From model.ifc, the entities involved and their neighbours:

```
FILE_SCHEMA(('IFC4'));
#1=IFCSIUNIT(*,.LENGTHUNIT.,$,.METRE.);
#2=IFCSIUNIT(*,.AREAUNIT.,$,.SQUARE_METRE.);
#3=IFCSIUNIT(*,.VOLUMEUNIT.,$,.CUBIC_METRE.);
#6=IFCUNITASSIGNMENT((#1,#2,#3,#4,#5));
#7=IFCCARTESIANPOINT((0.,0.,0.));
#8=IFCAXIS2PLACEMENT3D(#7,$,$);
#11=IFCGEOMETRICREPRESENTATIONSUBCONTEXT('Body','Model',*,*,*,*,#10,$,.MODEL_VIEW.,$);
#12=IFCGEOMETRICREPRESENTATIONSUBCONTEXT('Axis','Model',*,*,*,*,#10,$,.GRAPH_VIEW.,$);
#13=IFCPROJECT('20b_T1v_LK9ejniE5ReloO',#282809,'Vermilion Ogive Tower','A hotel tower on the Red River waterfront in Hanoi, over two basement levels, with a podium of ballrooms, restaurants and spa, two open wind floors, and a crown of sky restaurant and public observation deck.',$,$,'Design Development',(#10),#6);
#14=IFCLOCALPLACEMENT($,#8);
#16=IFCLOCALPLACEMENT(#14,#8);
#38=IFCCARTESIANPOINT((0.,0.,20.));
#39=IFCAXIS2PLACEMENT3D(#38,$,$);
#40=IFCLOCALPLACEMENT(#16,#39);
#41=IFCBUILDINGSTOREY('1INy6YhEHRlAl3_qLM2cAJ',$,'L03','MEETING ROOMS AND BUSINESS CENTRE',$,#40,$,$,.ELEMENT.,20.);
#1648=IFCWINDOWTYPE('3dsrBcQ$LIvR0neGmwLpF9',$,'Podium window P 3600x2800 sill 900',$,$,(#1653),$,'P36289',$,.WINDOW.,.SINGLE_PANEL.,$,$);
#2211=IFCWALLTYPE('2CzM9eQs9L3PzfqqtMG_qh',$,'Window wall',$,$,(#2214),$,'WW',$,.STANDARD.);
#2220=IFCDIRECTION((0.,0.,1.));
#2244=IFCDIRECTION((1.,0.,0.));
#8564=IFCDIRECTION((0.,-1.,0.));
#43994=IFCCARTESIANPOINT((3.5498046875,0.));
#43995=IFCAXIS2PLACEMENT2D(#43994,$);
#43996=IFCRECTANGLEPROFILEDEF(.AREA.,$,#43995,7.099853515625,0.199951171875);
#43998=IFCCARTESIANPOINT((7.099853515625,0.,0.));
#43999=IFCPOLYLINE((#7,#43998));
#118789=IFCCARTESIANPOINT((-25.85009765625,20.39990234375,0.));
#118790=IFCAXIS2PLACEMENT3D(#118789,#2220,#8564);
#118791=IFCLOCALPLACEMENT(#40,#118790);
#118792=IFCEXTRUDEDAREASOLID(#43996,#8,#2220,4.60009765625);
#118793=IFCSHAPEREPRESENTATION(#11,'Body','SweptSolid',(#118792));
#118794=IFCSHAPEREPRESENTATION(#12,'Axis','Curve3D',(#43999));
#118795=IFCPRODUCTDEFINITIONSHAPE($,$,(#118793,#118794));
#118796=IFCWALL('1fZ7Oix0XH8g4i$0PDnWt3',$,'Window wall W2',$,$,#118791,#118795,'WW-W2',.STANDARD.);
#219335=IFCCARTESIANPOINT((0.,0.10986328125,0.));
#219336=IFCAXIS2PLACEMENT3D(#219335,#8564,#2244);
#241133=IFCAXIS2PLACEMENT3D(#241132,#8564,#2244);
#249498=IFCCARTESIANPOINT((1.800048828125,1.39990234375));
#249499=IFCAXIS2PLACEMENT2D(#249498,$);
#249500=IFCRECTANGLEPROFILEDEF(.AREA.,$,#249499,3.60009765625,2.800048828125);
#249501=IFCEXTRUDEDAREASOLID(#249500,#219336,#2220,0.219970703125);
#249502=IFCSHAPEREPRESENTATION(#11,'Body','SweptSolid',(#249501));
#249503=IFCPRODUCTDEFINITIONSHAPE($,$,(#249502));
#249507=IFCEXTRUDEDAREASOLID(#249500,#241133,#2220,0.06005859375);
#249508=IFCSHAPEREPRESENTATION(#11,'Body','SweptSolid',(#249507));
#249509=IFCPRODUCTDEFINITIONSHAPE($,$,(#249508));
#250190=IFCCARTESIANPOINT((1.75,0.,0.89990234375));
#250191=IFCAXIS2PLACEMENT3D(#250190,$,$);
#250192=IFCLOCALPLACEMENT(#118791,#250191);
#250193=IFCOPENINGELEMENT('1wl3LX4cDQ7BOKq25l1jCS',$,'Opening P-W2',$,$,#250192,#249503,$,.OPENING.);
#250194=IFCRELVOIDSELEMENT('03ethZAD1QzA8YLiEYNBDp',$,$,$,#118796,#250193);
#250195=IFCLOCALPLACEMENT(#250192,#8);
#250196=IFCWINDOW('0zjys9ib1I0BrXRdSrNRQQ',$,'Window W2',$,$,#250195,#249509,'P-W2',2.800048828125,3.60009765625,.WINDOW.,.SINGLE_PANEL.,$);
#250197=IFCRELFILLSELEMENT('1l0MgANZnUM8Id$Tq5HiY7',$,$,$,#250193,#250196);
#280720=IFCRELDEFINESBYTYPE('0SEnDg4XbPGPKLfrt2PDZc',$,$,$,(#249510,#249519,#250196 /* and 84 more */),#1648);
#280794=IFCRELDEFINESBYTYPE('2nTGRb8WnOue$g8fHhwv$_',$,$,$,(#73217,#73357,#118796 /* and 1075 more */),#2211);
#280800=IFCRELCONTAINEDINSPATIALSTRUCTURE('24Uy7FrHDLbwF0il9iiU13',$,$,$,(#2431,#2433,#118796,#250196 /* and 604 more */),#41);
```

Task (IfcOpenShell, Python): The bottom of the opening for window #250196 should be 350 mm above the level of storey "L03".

```python
import numpy as np
import ifcopenshell
import ifcopenshell.api.geometry
import ifcopenshell.geom
import ifcopenshell.util.element
import ifcopenshell.util.placement
import ifcopenshell.util.shape
import ifcopenshell.util.unit

model = ifcopenshell.open("model.ifc")
unit_scale = ifcopenshell.util.unit.calculate_unit_scale(model)

window = model.by_id(250196)
opening = window.FillsVoids[0].RelatingOpeningElement
storey = ifcopenshell.util.element.get_container(window, ifc_class="IfcBuildingStorey")
level = ifcopenshell.util.placement.get_local_placement(storey.ObjectPlacement)[2, 3]

# The opening's origin need not be at the sill, so measure its lowest point.
shape = ifcopenshell.geom.create_shape(ifcopenshell.geom.settings(), opening)
bottom = ifcopenshell.util.shape.get_shape_bottom_elevation(shape, shape.geometry) / unit_scale
dz = level + 0.35 / unit_scale - bottom

shift = np.array([0.0, 0.0, dz])
# The window is placed relative to its opening, so it follows when the opening moves.
matrix = ifcopenshell.util.placement.get_local_placement(opening.ObjectPlacement)
matrix[:3, 3] += shift
ifcopenshell.api.geometry.edit_object_placement(
    model, product=opening, matrix=matrix, is_si=False, should_transform_children=True
)

print(f"moved by {dz * unit_scale:+.3f} m")

model.write("model-out.ifc")
```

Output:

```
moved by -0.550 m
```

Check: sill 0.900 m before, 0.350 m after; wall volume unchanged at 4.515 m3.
